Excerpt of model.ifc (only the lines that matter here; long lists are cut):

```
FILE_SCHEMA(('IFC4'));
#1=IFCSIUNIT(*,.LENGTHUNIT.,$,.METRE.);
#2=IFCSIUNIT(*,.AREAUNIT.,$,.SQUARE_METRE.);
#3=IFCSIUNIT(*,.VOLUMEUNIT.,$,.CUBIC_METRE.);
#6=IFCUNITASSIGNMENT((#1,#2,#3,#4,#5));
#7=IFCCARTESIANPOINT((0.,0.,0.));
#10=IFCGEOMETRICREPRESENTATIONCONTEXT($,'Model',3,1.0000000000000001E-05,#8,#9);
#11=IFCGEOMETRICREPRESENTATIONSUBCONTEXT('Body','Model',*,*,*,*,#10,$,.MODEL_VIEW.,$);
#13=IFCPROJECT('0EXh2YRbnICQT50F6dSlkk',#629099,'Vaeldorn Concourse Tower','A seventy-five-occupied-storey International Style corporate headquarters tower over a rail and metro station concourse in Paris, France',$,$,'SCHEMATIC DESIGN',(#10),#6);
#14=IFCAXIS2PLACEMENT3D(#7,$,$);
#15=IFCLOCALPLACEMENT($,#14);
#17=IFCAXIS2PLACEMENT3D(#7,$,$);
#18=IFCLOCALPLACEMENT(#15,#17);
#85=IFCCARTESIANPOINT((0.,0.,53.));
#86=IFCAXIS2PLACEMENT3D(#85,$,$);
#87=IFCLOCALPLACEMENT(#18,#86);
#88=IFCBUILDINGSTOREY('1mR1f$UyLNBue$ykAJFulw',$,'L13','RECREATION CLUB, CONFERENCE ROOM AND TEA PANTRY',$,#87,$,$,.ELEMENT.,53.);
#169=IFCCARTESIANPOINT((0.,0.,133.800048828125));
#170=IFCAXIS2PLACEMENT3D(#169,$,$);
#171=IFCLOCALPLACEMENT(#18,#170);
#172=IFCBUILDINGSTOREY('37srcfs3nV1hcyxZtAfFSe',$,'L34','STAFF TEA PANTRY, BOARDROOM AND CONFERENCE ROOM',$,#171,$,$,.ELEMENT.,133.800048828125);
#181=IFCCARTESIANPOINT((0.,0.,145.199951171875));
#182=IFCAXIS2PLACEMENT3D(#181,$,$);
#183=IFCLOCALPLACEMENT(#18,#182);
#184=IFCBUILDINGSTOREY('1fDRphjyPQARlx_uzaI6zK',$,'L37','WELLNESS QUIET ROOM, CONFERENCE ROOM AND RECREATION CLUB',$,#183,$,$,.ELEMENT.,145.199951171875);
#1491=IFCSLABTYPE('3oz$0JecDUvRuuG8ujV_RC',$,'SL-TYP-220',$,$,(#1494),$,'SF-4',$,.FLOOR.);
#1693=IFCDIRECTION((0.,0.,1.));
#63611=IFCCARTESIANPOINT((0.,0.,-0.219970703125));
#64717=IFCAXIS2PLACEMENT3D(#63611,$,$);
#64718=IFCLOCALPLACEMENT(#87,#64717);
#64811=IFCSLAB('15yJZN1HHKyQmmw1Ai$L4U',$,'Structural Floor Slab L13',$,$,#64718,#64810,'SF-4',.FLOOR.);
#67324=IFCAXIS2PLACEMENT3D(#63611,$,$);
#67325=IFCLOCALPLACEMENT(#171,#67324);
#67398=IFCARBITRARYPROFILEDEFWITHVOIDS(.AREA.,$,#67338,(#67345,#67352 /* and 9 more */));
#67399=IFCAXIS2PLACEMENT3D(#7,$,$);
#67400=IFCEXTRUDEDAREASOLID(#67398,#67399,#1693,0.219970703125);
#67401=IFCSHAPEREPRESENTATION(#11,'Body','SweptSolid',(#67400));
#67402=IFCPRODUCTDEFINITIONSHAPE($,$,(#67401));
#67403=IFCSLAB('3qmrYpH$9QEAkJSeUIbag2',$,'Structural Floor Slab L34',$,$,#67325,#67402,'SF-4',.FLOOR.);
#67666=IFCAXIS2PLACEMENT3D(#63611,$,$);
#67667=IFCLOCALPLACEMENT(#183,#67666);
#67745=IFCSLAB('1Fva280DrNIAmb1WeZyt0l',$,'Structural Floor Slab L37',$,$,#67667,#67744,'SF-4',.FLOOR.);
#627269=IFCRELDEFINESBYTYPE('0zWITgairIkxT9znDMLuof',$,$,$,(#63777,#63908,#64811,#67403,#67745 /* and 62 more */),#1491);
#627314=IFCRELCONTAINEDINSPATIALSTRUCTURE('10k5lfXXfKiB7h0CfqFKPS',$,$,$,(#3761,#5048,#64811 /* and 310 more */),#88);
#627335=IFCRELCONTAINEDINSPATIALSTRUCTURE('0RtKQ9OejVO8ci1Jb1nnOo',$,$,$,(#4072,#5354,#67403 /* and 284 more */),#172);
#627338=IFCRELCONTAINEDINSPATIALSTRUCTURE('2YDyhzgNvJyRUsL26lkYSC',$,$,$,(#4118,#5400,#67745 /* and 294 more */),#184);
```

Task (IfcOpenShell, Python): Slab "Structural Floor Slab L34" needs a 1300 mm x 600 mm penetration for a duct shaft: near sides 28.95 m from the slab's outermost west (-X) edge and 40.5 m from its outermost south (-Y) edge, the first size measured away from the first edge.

```python
import numpy as np
import ifcopenshell
import ifcopenshell.api.feature
import ifcopenshell.api.geometry
import ifcopenshell.api.root
import ifcopenshell.geom
import ifcopenshell.util.placement
import ifcopenshell.util.representation
import ifcopenshell.util.shape
import ifcopenshell.util.unit

model = ifcopenshell.open("model.ifc")
unit_scale = ifcopenshell.util.unit.calculate_unit_scale(model)
settings = ifcopenshell.geom.settings()


def volume(element):
    """Net volume in cubic metres, openings subtracted."""
    shape = ifcopenshell.geom.create_shape(settings, element)
    return ifcopenshell.util.shape.get_volume(shape.geometry)


slab = model.by_guid("3qmrYpH$9QEAkJSeUIbag2")
before = volume(slab)

# Extent in the slab's own axes, in metres. The edges named are its -X and -Y sides.
slab_shape = ifcopenshell.geom.create_shape(settings, slab)
vertices = ifcopenshell.util.shape.get_vertices(slab_shape.geometry)
x_min, y_min, bottom = vertices.min(axis=0)
top = vertices[:, 2].max()

opening = ifcopenshell.api.root.create_entity(model, ifc_class="IfcOpeningElement", name="Duct shaft opening", predefined_type="OPENING")
context = ifcopenshell.util.representation.get_context(model, "Model", "Body", "MODEL_VIEW")
width, depth = 1.3, 0.6
outline = [(0.0, 0.0), (width, 0.0), (width, depth), (0.0, depth), (0.0, 0.0)]
# Overshoot both faces by 50 mm so the cut is clean.
shape = ifcopenshell.api.geometry.add_slab_representation(
    model, context=context, depth=top - bottom + 0.1, polyline=outline
)
ifcopenshell.api.geometry.assign_representation(model, product=opening, representation=shape)

matrix = ifcopenshell.util.placement.get_local_placement(slab.ObjectPlacement)
matrix[:, 3] = matrix @ np.append(np.array([x_min + 28.95, y_min + 40.5, bottom - 0.05]) / unit_scale, 1.0)
ifcopenshell.api.geometry.edit_object_placement(model, product=opening, matrix=matrix, is_si=False)
ifcopenshell.api.feature.add_feature(model, feature=opening, element=slab)

after = volume(slab)

print(f"slab volume {before:.3f} -> {after:.3f} m3")

model.write("model_rev.ifc")
```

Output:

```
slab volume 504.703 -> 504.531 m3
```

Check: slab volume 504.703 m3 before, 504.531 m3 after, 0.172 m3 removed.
